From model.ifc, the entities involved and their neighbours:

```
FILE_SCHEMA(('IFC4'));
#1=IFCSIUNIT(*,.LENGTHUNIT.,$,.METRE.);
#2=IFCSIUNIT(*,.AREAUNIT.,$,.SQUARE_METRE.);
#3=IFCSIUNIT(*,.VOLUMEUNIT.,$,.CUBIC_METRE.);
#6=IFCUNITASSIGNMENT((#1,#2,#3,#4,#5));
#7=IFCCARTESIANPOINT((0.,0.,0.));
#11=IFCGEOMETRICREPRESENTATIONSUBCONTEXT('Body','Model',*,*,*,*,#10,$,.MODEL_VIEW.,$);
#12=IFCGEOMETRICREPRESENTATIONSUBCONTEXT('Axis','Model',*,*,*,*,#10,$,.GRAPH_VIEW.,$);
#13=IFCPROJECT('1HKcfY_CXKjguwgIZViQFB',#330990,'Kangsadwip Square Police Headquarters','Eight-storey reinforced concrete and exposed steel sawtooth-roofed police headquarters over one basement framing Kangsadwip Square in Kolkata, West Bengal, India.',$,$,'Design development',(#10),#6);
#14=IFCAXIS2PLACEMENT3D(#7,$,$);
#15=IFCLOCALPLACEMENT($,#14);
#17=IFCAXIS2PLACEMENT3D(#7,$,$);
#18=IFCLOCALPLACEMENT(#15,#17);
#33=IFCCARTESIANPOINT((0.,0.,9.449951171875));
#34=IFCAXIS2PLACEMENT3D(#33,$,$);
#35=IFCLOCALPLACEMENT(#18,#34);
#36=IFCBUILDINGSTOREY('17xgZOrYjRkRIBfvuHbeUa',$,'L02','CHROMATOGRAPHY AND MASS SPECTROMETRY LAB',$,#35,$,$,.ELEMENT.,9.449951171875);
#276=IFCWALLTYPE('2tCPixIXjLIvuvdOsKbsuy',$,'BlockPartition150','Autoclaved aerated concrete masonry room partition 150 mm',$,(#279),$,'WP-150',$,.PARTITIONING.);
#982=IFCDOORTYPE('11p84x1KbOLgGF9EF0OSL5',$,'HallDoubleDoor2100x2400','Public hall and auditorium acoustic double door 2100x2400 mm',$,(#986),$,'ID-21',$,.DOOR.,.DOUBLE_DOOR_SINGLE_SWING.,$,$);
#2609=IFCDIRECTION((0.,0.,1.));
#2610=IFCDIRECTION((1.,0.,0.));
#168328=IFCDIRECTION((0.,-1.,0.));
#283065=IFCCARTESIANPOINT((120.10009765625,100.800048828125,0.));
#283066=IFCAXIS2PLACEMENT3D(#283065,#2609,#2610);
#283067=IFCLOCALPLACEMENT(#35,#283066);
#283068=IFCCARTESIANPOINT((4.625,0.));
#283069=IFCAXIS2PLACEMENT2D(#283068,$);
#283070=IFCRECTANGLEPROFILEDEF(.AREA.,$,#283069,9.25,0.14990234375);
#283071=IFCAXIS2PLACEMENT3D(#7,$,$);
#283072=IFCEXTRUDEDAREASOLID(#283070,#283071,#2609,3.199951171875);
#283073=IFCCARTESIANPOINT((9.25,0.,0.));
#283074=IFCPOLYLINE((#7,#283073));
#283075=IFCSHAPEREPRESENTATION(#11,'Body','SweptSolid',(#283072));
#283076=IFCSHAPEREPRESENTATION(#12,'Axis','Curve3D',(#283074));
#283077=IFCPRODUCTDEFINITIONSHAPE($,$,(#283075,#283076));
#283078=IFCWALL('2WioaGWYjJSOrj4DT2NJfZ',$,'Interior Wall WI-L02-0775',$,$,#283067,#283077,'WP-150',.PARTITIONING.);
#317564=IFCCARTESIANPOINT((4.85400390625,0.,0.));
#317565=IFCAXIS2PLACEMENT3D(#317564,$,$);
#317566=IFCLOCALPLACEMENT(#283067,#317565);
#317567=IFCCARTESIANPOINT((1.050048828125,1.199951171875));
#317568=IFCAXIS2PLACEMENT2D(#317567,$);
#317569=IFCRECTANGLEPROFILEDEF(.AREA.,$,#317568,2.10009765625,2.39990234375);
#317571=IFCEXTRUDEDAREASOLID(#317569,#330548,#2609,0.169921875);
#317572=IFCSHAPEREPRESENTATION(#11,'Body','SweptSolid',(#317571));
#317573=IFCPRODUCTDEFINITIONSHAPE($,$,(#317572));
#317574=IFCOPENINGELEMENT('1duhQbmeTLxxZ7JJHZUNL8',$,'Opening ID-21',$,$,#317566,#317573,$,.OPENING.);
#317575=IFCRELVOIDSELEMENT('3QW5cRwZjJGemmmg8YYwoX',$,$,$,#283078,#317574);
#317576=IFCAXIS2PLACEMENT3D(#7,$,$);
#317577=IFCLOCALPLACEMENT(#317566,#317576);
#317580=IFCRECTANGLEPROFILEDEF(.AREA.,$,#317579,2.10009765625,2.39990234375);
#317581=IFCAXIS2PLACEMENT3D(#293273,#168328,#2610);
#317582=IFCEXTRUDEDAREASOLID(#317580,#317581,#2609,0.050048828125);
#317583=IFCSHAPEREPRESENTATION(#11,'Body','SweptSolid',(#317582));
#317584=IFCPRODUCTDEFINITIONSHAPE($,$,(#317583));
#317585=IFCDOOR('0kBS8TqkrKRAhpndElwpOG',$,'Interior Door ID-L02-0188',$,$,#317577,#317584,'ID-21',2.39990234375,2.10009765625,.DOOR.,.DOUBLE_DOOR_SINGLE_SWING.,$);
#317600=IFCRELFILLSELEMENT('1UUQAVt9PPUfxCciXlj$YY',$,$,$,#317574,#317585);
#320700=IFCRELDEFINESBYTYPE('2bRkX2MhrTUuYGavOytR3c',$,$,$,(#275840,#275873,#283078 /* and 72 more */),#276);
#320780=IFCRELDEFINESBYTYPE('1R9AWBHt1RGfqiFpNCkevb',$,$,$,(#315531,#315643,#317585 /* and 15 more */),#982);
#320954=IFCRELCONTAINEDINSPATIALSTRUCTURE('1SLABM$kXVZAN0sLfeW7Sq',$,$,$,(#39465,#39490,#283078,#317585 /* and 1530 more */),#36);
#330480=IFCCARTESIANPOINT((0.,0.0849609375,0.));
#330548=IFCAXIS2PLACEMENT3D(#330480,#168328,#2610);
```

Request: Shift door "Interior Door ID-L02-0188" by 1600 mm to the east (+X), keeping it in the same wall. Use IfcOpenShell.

```python
import ifcopenshell
import ifcopenshell.api.geometry
import ifcopenshell.util.placement
import ifcopenshell.util.unit

model = ifcopenshell.open("model.ifc")
unit_scale = ifcopenshell.util.unit.calculate_unit_scale(model)

door = model.by_guid("0kBS8TqkrKRAhpndElwpOG")
opening = door.FillsVoids[0].RelatingOpeningElement
wall = opening.VoidsElements[0].RelatingBuildingElement

wall_matrix = ifcopenshell.util.placement.get_local_placement(wall.ObjectPlacement)
shift = wall_matrix[:3, 0] * 1.6 / unit_scale
before = ifcopenshell.util.placement.get_local_placement(door.ObjectPlacement)[:3, 3].copy()

# The door is placed relative to its opening, so it follows when the opening moves.
matrix = ifcopenshell.util.placement.get_local_placement(opening.ObjectPlacement)
matrix[:3, 3] += shift
ifcopenshell.api.geometry.edit_object_placement(
    model, product=opening, matrix=matrix, is_si=False, should_transform_children=True
)

after = ifcopenshell.util.placement.get_local_placement(door.ObjectPlacement)[:3, 3]
print("door moved by", (after - before).round(3) + 0.0)

model.write("model_updated.ifc")
```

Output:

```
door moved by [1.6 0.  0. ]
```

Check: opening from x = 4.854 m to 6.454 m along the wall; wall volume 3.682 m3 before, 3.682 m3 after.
